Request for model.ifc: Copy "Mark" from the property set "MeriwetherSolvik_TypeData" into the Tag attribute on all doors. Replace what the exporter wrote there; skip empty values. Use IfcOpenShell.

First a look at what the model holds.

```python
import ifcopenshell
import ifcopenshell.util.element

model = ifcopenshell.open("model.ifc")
print(model.schema)
doors = model.by_type("IfcDoor")
print(len(doors), "doors")
for e in doors[:8]:
    source = ifcopenshell.util.element.get_pset(e, "MeriwetherSolvik_TypeData", "Mark")
    target = e.Tag
    print(e.id(), repr(source), repr(target), sep=" | ")
```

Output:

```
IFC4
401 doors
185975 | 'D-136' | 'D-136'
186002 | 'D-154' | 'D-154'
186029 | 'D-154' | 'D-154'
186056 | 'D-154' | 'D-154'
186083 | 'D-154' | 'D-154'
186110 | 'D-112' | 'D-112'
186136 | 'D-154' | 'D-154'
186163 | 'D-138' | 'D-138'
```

```python
import ifcopenshell
import ifcopenshell.util.element

model = ifcopenshell.open("model.ifc")

count = 0
for e in model.by_type("IfcDoor"):
    value = ifcopenshell.util.element.get_pset(e, "MeriwetherSolvik_TypeData", "Mark")
    current = e.Tag
    if not value or not value.strip() or current == value:
        continue
    e.Tag = value
    count += 1

print(count, "doors updated")

model.write("model_v2.ifc")
```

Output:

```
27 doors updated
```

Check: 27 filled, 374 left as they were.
